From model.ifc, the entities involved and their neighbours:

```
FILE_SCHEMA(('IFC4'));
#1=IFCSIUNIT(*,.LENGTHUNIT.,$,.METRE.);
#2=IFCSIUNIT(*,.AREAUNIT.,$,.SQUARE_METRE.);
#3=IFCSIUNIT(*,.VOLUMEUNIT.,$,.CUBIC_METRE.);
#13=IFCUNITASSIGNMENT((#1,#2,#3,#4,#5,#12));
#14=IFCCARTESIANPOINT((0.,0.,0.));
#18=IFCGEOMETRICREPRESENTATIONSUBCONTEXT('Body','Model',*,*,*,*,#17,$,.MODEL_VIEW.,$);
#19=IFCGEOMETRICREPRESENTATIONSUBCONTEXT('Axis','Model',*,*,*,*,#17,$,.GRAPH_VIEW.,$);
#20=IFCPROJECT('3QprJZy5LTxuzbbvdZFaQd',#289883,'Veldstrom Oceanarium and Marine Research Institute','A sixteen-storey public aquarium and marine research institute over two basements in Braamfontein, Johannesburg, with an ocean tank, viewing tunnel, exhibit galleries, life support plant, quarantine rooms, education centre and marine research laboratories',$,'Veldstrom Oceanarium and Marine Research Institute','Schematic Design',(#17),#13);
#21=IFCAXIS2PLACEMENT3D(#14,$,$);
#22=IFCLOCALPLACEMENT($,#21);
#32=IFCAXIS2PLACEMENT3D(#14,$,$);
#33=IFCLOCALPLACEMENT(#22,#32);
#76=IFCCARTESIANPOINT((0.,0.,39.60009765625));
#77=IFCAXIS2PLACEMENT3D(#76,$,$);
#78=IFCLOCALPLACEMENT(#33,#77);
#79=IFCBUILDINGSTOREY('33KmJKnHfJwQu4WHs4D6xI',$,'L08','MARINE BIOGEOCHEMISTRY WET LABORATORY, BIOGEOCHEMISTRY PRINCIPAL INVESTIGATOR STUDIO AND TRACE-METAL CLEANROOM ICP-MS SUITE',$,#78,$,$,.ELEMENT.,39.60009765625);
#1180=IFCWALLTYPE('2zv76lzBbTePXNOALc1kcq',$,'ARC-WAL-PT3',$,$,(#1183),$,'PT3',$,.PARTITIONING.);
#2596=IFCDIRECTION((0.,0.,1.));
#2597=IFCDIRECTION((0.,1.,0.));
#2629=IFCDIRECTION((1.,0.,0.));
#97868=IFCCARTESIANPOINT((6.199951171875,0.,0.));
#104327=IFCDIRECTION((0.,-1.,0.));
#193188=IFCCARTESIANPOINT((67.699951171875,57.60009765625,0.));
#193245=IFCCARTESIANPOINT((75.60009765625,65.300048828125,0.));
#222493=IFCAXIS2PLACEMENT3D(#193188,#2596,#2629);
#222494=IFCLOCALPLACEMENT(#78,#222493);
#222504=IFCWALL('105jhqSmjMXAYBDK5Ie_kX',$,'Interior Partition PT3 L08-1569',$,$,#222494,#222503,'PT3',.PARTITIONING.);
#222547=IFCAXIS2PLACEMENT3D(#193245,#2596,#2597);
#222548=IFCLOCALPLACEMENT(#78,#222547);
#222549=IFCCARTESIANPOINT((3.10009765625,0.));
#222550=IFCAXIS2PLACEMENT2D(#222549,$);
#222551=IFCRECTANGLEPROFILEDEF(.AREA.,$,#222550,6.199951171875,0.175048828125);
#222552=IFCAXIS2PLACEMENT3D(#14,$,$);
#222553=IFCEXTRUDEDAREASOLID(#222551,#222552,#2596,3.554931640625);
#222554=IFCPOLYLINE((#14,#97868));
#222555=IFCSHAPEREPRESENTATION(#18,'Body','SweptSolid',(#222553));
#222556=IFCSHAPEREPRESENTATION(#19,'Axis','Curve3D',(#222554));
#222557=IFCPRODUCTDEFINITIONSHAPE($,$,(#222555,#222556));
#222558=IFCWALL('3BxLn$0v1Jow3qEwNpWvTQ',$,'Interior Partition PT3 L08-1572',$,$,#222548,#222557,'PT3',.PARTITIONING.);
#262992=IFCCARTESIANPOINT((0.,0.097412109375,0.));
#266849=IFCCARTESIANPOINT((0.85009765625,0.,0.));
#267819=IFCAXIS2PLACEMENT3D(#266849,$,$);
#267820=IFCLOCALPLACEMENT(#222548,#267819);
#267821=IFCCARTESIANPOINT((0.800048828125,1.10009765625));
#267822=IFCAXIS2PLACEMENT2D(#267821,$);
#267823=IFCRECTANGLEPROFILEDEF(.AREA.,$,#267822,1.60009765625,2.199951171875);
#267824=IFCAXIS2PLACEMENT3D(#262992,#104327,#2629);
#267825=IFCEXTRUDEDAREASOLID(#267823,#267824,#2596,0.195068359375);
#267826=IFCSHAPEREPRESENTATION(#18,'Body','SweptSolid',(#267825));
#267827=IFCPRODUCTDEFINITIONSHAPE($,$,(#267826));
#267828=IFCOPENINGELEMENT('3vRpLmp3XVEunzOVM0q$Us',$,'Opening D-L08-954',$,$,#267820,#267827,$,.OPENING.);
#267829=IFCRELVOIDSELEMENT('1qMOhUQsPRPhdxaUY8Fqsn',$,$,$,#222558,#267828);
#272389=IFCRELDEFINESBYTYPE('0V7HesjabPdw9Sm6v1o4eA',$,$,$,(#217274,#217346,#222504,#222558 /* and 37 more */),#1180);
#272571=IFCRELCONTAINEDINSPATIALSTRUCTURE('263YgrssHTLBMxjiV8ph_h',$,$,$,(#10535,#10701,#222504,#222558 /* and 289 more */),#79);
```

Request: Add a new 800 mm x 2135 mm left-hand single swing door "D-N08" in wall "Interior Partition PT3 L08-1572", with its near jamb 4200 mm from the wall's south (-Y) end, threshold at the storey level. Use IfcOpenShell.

```python
import numpy as np
import ifcopenshell
import ifcopenshell.api.feature
import ifcopenshell.api.geometry
import ifcopenshell.api.root
import ifcopenshell.api.spatial
import ifcopenshell.geom
import ifcopenshell.util.element
import ifcopenshell.util.placement
import ifcopenshell.util.representation
import ifcopenshell.util.shape
import ifcopenshell.util.unit

model = ifcopenshell.open("model.ifc")
unit_scale = ifcopenshell.util.unit.calculate_unit_scale(model)
settings = ifcopenshell.geom.settings()


def volume(element):
    """Net volume in cubic metres, openings subtracted."""
    shape = ifcopenshell.geom.create_shape(settings, element)
    return ifcopenshell.util.shape.get_volume(shape.geometry)


wall = model.by_guid("3BxLn$0v1Jow3qEwNpWvTQ")
storey = ifcopenshell.util.element.get_container(wall, ifc_class="IfcBuildingStorey")
context = ifcopenshell.util.representation.get_context(model, "Model", "Body", "MODEL_VIEW")
before = volume(wall)

width, height, from_end, sill = 0.8, 2.135, 4.2, 0.0  # metres

# The wall runs along its own X axis, and the end named is its -X end.
wall_shape = ifcopenshell.geom.create_shape(settings, wall)
x, y, z = ifcopenshell.util.shape.get_vertices(wall_shape.geometry).T
start = x.min() + from_end
face, thickness = float(y.min()), float(y.max() - y.min())
wall_matrix = ifcopenshell.util.placement.get_local_placement(wall.ObjectPlacement)
level = ifcopenshell.util.placement.get_local_placement(storey.ObjectPlacement)[2, 3]


def in_wall(x, y):
    """Placement at x, y metres in the wall's axes, at sill height."""
    matrix = wall_matrix.copy()
    matrix[:, 3] = wall_matrix @ np.array([x / unit_scale, y / unit_scale, 0.0, 1.0])
    matrix[2, 3] = level + sill / unit_scale
    return matrix


# Opening: a box that overshoots both wall faces by 50 mm.
opening = ifcopenshell.api.root.create_entity(model, ifc_class="IfcOpeningElement", predefined_type="OPENING")
box = ifcopenshell.api.geometry.add_wall_representation(
    model, context=context, length=width, height=height, thickness=thickness + 0.1
)
ifcopenshell.api.geometry.assign_representation(model, product=opening, representation=box)
ifcopenshell.api.geometry.edit_object_placement(model, product=opening, matrix=in_wall(start, face - 0.05), is_si=False)
ifcopenshell.api.feature.add_feature(model, feature=opening, element=wall)

door = ifcopenshell.api.root.create_entity(model, ifc_class="IfcDoor", name="D-N08", predefined_type="DOOR")
door.OverallWidth, door.OverallHeight = width / unit_scale, height / unit_scale
door.OperationType = "SINGLE_SWING_LEFT"
body = ifcopenshell.api.geometry.add_door_representation(
    model,
    context=context,
    overall_width=door.OverallWidth,
    overall_height=door.OverallHeight,
    operation_type="SINGLE_SWING_LEFT",
    lining_properties={"LiningDepth": thickness / unit_scale, "ThresholdDepth": thickness / unit_scale},
)
ifcopenshell.api.geometry.assign_representation(model, product=door, representation=body)
ifcopenshell.api.spatial.assign_container(model, products=[door], relating_structure=storey)
ifcopenshell.api.feature.add_filling(model, opening=opening, element=door)

# The lining spans the wall, so the door starts at the wall face.
ifcopenshell.api.geometry.edit_object_placement(model, product=door, matrix=in_wall(start, face), is_si=False)

after = volume(wall)

print(f"wall volume {before:.3f} -> {after:.3f} m3")

model.write("model_edited.ifc")
```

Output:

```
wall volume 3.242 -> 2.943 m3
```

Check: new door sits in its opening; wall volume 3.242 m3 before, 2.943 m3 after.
